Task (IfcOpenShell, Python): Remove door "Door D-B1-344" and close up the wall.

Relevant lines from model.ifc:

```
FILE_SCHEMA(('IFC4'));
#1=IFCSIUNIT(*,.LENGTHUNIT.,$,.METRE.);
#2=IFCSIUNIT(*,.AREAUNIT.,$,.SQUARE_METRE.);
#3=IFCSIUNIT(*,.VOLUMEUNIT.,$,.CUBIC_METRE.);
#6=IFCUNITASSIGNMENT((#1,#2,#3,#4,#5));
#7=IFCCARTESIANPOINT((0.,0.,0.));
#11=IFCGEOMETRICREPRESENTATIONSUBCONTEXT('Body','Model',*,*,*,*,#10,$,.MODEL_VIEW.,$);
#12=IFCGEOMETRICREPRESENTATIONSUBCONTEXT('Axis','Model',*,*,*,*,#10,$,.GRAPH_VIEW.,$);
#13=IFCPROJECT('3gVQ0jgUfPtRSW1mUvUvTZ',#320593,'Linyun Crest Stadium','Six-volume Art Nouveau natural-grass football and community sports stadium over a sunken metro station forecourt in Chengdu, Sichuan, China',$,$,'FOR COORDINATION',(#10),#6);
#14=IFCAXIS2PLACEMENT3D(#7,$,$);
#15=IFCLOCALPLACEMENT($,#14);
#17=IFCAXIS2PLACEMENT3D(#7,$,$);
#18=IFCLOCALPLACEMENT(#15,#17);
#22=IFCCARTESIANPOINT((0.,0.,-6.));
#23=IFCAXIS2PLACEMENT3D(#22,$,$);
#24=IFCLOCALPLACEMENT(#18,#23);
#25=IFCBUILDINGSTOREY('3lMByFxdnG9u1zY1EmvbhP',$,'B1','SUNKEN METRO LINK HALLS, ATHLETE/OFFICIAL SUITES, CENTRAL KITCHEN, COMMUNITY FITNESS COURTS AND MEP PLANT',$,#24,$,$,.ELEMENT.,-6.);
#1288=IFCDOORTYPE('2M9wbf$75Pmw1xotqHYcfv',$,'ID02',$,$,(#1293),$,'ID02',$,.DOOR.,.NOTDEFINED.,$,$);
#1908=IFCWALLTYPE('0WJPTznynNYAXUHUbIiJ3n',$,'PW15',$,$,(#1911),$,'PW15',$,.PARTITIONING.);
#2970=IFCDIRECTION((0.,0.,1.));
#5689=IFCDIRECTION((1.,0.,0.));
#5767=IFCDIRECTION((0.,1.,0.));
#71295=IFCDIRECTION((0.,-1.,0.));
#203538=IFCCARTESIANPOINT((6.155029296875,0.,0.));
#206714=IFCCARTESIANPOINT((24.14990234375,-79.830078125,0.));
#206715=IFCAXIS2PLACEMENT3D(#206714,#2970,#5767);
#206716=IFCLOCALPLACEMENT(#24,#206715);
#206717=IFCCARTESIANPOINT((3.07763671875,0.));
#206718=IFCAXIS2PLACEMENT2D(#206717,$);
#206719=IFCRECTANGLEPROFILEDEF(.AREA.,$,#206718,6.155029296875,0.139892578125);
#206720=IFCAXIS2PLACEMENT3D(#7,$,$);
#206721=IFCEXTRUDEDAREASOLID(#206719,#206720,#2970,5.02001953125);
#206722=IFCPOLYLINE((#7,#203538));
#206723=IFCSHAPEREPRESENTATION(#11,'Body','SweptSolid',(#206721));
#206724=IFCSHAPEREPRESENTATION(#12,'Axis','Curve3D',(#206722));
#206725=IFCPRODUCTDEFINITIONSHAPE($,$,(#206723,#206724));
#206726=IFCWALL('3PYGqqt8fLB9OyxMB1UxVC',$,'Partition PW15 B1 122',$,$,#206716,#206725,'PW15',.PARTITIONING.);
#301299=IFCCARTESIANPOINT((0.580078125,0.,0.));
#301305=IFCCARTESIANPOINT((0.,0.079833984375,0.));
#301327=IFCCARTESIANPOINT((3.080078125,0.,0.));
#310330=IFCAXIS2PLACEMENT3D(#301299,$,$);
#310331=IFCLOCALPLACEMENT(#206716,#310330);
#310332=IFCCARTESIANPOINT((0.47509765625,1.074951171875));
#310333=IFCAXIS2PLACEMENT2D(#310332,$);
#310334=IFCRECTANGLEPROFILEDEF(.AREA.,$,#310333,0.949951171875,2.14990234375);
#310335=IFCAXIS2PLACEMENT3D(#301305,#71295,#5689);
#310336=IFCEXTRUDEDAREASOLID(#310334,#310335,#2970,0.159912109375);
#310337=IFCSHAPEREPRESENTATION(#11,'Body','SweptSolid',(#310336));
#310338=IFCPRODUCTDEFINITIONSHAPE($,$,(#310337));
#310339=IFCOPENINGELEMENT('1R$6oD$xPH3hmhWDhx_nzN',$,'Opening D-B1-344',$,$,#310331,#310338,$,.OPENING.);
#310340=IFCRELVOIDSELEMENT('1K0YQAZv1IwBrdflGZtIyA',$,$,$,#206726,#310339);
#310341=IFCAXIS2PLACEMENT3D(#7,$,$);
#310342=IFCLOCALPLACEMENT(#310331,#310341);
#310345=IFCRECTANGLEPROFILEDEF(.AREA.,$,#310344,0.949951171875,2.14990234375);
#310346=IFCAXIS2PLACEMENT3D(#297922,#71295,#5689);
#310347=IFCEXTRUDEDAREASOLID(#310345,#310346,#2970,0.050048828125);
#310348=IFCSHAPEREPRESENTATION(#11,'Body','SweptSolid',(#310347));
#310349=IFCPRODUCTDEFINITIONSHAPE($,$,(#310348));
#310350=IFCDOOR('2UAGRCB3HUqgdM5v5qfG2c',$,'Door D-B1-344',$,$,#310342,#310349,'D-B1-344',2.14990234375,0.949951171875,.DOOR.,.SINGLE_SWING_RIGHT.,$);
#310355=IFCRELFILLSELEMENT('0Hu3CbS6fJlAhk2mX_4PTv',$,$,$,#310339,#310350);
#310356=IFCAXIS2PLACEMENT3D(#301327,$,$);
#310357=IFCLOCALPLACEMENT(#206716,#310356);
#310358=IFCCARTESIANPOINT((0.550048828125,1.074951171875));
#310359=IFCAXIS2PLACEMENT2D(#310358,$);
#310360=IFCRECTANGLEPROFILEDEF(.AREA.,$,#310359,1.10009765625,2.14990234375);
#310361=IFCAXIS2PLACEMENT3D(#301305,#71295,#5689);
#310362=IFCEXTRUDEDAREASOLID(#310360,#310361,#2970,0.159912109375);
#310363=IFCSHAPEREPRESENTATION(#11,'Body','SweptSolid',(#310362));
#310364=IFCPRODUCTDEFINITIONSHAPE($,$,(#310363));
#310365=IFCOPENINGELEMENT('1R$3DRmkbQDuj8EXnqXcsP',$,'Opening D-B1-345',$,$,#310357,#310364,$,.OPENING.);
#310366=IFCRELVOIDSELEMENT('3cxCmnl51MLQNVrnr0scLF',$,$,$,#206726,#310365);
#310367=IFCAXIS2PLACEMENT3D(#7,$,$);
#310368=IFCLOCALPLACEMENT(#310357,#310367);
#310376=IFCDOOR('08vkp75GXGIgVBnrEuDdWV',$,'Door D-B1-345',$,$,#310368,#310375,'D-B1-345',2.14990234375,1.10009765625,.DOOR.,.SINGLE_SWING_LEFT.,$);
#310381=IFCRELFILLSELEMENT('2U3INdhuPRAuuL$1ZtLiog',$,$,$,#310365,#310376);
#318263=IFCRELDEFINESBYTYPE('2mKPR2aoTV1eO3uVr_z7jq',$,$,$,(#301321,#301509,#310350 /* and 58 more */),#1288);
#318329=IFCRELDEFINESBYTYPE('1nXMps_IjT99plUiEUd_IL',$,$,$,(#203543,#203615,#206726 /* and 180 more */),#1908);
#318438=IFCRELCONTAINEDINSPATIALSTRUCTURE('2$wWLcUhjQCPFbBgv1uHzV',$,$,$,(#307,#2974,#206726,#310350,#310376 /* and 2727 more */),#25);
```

```python
import ifcopenshell
import ifcopenshell.api.feature
import ifcopenshell.api.root
import ifcopenshell.geom
import ifcopenshell.util.shape

model = ifcopenshell.open("model.ifc")
settings = ifcopenshell.geom.settings()


def volume(element):
    """Net volume in cubic metres, openings subtracted."""
    shape = ifcopenshell.geom.create_shape(settings, element)
    return ifcopenshell.util.shape.get_volume(shape.geometry)


door = model.by_id(310350)
opening = door.FillsVoids[0].RelatingOpeningElement
wall = opening.VoidsElements[0].RelatingBuildingElement
before = volume(wall)

ifcopenshell.api.root.remove_product(model, product=door)
ifcopenshell.api.feature.remove_feature(model, feature=opening)

after = volume(wall)

print(f"wall volume {before:.3f} -> {after:.3f} m3")

model.write("model_edited.ifc")
```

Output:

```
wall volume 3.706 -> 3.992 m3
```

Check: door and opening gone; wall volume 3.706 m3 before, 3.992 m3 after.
